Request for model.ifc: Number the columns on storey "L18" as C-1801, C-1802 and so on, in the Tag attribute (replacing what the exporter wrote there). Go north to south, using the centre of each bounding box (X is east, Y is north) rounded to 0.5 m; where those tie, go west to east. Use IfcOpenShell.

First a look at what the model holds.

```python
import ifcopenshell
import ifcopenshell.util.element
import ifcopenshell.util.placement

model = ifcopenshell.open("model.ifc")
print(model.schema)
storey = next(s for s in model.by_type("IfcBuildingStorey") if s.Name == "L18")
columns = [e for e in ifcopenshell.util.element.get_decomposition(storey) if e.is_a("IfcColumn")]
for e in sorted(columns, key=lambda e: e.id()):
    origin = ifcopenshell.util.placement.get_local_placement(e.ObjectPlacement)[:3, 3]
    print(e.id(), e.Tag, e.Name, origin.round(2) + 0.0, sep=" | ")
```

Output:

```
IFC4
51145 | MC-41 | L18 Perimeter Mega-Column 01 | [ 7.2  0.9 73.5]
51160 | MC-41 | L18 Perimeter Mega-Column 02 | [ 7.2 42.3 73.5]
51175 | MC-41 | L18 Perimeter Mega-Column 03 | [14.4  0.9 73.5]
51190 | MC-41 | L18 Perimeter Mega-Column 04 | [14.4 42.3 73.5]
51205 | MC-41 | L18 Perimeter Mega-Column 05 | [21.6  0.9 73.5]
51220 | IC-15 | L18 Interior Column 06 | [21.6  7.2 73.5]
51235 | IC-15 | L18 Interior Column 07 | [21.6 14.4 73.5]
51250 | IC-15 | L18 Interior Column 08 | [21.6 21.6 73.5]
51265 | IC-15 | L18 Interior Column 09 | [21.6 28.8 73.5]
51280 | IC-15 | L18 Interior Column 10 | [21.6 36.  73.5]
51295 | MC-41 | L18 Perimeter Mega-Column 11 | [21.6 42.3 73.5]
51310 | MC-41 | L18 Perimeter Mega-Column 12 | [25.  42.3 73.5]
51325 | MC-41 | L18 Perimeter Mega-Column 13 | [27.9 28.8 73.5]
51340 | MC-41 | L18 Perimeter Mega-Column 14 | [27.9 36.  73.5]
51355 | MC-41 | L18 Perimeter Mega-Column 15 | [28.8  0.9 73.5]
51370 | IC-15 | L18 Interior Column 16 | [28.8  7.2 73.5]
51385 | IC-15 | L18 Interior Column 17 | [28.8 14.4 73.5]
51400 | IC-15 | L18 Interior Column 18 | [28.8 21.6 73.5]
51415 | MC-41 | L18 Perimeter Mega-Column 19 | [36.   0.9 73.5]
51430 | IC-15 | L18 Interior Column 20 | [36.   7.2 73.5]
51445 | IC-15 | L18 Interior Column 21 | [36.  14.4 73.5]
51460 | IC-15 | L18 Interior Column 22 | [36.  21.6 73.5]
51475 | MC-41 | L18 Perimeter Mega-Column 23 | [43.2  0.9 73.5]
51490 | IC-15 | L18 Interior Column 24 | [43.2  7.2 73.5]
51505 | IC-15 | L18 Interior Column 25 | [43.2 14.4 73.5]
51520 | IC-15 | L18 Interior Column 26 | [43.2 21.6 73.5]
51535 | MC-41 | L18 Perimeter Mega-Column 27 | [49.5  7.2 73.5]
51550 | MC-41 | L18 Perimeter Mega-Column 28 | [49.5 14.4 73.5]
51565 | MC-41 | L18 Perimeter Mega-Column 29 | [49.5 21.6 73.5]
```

```python
import ifcopenshell
import ifcopenshell.geom
import ifcopenshell.util.element
import ifcopenshell.util.shape

model = ifcopenshell.open("model.ifc")
settings = ifcopenshell.geom.settings()
settings.set("use-world-coords", True)


def centre(element):
    shape = ifcopenshell.geom.create_shape(settings, element)
    return ifcopenshell.util.shape.get_bbox_centroid(shape.geometry)


storey = next(s for s in model.by_type("IfcBuildingStorey") if s.Name == "L18")
columns = [e for e in ifcopenshell.util.element.get_decomposition(storey) if e.is_a("IfcColumn")]

# Insertion points can sit at a corner or the storey origin, so sort by the geometry (in metres).
centres = {e: centre(e) for e in columns}
columns.sort(key=lambda e: (-round(centres[e][1] / 0.5), centres[e][0]))

for i, e in enumerate(columns, start=1):
    number = f"C-18{i:02d}"
    e.Tag = number
    print(e.id(), number)

model.write("model_updated.ifc")
```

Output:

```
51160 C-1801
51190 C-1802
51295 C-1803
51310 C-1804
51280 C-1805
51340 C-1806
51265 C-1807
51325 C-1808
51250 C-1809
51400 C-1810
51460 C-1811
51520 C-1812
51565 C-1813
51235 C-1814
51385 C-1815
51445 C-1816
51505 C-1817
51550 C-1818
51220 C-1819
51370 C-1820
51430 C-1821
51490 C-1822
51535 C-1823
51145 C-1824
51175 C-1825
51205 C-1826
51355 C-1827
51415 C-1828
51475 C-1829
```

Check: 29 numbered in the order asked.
